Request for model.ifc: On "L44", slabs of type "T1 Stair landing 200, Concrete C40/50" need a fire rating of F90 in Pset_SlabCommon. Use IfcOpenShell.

First a look at what the model holds.

```python
import ifcopenshell
import ifcopenshell.util.element

model = ifcopenshell.open("model.ifc")
print(model.schema)
storey = next(s for s in model.by_type("IfcBuildingStorey") if s.Name == "L44")
slabs = [e for e in ifcopenshell.util.element.get_decomposition(storey) if e.is_a("IfcSlab")]
seen = {}
for e in slabs:
    element_type = ifcopenshell.util.element.get_type(e)
    key = (element_type.Name if element_type != e and element_type else None, ifcopenshell.util.element.get_pset(e, "Pset_SlabCommon", "FireRating"))
    seen[key] = seen.get(key, 0) + 1
for (name, value), count in sorted(seen.items(), key=str):
    print(count, "x", name, "|", value)
```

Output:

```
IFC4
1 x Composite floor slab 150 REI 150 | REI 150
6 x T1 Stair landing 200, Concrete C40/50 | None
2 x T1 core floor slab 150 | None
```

```python
import ifcopenshell
import ifcopenshell.api.pset
import ifcopenshell.util.element

model = ifcopenshell.open("model.ifc")

storey = next(s for s in model.by_type("IfcBuildingStorey") if s.Name == "L44")
slabs = [e for e in ifcopenshell.util.element.get_decomposition(storey) if e.is_a("IfcSlab")]

count = 0
for e in slabs:
    element_type = ifcopenshell.util.element.get_type(e)
    if element_type in (None, e) or element_type.Name != "T1 Stair landing 200, Concrete C40/50":
        continue
    found = ifcopenshell.util.element.get_pset(e, "Pset_SlabCommon", should_inherit=False)
    if found:
        pset = model.by_id(found["id"])
        if len(ifcopenshell.util.element.get_elements_by_pset(pset)) > 1:
            pset = ifcopenshell.api.pset.unshare_pset(model, products=[e], pset=pset)[0]
    else:
        pset = ifcopenshell.api.pset.add_pset(model, product=e, name="Pset_SlabCommon")
    ifcopenshell.api.pset.edit_pset(model, pset=pset, properties={"FireRating": "F90"})
    count += 1

print(count, "slabs updated")

model.write("model_v2.ifc")
```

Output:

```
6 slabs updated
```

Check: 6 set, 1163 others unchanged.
